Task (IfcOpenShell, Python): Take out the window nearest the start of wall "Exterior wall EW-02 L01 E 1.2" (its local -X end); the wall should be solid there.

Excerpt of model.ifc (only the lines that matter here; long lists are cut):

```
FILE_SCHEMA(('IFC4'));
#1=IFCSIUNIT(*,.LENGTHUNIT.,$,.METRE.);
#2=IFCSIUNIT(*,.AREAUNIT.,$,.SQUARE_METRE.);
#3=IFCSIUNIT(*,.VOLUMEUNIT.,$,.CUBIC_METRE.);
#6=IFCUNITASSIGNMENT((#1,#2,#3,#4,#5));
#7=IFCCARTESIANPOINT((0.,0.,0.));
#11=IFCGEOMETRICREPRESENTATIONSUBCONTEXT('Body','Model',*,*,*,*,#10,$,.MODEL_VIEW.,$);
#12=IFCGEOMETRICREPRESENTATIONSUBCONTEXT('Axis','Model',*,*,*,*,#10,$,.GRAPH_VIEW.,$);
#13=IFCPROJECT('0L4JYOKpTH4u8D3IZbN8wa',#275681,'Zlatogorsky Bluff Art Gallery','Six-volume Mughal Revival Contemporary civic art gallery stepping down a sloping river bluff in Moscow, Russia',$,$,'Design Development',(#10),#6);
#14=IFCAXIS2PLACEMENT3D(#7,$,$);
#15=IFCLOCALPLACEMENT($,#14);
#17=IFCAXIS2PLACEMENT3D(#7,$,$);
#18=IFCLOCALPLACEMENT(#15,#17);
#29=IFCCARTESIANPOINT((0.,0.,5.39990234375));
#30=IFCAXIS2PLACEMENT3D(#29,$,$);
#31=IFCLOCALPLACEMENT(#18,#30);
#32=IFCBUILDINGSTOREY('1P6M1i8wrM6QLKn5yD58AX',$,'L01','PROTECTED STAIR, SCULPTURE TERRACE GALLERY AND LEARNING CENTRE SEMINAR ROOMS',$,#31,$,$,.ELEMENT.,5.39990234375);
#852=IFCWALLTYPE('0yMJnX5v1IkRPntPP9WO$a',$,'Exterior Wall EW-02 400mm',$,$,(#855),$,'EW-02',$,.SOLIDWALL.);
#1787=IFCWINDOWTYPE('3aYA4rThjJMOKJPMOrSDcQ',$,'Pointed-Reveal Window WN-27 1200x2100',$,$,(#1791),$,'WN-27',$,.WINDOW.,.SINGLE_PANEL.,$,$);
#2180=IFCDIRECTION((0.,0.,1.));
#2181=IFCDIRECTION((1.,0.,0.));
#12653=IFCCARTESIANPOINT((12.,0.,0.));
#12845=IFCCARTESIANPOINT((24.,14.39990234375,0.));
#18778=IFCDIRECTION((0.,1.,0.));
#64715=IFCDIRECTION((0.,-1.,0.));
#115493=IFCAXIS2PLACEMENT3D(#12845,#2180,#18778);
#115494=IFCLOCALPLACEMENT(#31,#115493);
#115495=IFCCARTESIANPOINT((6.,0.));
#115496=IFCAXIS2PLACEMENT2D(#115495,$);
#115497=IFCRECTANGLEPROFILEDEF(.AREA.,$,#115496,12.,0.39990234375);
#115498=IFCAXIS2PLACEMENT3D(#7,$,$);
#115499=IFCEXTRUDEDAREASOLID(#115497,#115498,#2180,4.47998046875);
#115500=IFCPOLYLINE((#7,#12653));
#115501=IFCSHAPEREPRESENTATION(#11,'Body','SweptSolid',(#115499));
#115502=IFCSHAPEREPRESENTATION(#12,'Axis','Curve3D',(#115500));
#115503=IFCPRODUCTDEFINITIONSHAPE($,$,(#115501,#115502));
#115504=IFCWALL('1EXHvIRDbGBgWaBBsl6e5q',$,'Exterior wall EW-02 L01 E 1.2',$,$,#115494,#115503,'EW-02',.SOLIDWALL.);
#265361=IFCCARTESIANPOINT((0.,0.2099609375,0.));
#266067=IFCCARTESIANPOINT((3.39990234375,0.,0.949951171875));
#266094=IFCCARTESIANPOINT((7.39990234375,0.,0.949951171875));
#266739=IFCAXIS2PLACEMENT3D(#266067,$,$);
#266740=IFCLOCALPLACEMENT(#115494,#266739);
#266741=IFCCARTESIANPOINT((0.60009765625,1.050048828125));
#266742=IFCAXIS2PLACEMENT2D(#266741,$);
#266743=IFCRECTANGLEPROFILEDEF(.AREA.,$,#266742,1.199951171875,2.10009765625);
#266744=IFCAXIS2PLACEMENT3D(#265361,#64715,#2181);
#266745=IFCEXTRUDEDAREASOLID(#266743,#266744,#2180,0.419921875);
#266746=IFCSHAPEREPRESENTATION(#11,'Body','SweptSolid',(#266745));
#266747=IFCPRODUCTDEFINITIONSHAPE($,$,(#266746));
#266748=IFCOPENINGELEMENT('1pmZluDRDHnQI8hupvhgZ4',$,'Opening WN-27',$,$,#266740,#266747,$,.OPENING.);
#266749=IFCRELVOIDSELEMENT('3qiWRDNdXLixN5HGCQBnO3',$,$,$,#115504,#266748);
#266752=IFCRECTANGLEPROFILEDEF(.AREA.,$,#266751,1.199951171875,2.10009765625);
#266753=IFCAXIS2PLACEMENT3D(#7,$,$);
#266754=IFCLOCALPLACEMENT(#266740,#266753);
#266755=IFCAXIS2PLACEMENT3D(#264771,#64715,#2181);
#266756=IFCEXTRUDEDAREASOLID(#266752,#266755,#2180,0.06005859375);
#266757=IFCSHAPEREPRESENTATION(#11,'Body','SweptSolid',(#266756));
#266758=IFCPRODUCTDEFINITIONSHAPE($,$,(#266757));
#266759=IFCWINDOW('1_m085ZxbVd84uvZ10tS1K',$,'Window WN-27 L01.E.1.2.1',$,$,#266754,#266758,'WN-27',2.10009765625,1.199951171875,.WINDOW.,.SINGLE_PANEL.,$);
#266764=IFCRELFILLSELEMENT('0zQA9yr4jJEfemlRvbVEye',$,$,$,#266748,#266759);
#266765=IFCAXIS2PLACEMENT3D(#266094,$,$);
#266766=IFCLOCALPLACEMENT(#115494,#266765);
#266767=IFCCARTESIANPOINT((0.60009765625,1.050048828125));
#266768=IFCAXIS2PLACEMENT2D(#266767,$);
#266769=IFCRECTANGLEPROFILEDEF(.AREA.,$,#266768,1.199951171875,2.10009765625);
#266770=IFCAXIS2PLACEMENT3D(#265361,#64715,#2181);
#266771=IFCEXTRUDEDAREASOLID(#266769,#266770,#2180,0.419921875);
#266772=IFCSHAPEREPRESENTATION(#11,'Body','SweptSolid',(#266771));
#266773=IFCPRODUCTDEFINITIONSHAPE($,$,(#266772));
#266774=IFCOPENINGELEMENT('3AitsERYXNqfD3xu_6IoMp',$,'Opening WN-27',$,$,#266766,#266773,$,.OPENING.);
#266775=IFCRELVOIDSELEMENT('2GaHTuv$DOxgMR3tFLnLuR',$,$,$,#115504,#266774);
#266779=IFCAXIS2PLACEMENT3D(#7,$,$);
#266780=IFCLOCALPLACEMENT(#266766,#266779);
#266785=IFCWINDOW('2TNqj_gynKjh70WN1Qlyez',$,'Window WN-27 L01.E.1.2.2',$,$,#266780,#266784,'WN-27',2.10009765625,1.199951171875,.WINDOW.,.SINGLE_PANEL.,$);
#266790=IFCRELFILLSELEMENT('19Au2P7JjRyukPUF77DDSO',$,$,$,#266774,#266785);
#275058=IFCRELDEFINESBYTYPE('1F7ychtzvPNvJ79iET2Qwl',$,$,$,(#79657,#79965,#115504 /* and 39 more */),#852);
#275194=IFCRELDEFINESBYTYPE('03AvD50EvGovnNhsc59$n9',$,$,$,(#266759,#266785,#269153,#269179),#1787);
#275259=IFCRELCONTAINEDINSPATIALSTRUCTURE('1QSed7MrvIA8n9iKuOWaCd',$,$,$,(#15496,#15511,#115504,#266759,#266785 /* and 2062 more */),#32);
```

```python
import ifcopenshell
import ifcopenshell.api.feature
import ifcopenshell.api.root
import ifcopenshell.geom
import ifcopenshell.util.shape

model = ifcopenshell.open("model.ifc")
settings = ifcopenshell.geom.settings()


def volume(element):
    """Net volume in cubic metres, openings subtracted."""
    shape = ifcopenshell.geom.create_shape(settings, element)
    return ifcopenshell.util.shape.get_volume(shape.geometry)


window = model.by_id(266759)
opening = window.FillsVoids[0].RelatingOpeningElement
wall = opening.VoidsElements[0].RelatingBuildingElement
before = volume(wall)

ifcopenshell.api.root.remove_product(model, product=window)
ifcopenshell.api.feature.remove_feature(model, feature=opening)

after = volume(wall)

print(f"wall volume {before:.3f} -> {after:.3f} m3")

model.write("model_rev.ifc")
```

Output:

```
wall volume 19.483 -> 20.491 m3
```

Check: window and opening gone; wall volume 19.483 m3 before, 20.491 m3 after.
